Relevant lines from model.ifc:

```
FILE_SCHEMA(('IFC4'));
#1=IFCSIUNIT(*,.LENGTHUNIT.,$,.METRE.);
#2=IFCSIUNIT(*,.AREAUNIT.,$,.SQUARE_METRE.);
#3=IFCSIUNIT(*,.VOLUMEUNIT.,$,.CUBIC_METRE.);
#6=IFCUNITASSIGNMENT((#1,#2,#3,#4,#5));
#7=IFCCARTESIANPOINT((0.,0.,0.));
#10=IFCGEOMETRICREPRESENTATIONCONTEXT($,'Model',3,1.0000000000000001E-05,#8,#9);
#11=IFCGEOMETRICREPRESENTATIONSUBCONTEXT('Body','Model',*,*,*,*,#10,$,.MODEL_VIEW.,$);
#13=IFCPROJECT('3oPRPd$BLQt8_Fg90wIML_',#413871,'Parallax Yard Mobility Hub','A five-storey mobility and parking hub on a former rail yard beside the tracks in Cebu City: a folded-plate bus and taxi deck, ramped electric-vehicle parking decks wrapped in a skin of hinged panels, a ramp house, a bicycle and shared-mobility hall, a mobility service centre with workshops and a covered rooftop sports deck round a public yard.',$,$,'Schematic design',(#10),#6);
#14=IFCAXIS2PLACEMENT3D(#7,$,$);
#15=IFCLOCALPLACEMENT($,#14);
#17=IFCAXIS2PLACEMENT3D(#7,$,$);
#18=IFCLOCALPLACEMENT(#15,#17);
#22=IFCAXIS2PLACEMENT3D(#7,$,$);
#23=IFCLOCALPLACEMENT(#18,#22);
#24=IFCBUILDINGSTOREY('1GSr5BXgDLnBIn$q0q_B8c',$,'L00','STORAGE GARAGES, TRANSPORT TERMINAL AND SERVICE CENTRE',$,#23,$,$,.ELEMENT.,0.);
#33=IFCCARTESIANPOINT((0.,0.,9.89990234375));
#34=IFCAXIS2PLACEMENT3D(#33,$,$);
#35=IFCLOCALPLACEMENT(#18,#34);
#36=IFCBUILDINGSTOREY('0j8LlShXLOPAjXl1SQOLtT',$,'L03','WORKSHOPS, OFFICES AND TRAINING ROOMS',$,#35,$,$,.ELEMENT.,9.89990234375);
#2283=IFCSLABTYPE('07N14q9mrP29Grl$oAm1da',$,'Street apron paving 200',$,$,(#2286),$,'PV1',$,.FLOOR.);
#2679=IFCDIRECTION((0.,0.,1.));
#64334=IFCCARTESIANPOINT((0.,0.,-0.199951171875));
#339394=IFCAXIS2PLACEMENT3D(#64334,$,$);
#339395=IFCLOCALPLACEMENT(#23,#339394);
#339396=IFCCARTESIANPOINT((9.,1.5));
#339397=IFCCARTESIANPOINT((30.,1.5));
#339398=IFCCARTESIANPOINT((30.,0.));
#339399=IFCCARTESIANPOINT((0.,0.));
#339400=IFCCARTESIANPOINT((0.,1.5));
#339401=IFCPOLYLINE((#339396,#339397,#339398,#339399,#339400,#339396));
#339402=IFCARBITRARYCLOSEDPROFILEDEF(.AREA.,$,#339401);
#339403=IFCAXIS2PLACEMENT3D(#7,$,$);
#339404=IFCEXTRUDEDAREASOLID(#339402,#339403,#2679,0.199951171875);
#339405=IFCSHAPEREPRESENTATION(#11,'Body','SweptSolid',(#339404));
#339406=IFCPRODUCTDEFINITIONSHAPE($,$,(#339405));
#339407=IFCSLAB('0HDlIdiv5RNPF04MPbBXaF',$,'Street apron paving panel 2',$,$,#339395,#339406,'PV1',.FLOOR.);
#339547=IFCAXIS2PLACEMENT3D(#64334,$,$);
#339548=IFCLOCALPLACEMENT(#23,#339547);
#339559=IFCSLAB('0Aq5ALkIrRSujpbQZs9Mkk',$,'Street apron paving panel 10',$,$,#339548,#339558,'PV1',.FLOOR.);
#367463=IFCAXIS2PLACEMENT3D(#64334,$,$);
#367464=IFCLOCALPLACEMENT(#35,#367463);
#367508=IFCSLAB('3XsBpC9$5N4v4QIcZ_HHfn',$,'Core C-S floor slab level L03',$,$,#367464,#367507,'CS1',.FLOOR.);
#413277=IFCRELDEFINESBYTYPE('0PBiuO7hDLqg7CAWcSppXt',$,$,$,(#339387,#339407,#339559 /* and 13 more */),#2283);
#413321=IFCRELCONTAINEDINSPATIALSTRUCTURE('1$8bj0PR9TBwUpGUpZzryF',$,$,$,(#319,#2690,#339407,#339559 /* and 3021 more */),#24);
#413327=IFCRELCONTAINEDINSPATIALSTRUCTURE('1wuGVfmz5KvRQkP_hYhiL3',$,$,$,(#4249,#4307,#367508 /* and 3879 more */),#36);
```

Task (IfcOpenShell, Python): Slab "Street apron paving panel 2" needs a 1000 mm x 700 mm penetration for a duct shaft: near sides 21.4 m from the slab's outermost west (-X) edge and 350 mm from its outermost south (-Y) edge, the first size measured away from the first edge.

```python
import numpy as np
import ifcopenshell
import ifcopenshell.api.feature
import ifcopenshell.api.geometry
import ifcopenshell.api.root
import ifcopenshell.geom
import ifcopenshell.util.placement
import ifcopenshell.util.representation
import ifcopenshell.util.shape
import ifcopenshell.util.unit

model = ifcopenshell.open("model.ifc")
unit_scale = ifcopenshell.util.unit.calculate_unit_scale(model)
settings = ifcopenshell.geom.settings()


def volume(element):
    """Net volume in cubic metres, openings subtracted."""
    shape = ifcopenshell.geom.create_shape(settings, element)
    return ifcopenshell.util.shape.get_volume(shape.geometry)


slab = model.by_guid("0HDlIdiv5RNPF04MPbBXaF")
before = volume(slab)

# Extent in the slab's own axes, in metres. The edges named are its -X and -Y sides.
slab_shape = ifcopenshell.geom.create_shape(settings, slab)
vertices = ifcopenshell.util.shape.get_vertices(slab_shape.geometry)
x_min, y_min, bottom = vertices.min(axis=0)
top = vertices[:, 2].max()

opening = ifcopenshell.api.root.create_entity(model, ifc_class="IfcOpeningElement", name="Duct shaft opening", predefined_type="OPENING")
context = ifcopenshell.util.representation.get_context(model, "Model", "Body", "MODEL_VIEW")
width, depth = 1, 0.7
outline = [(0.0, 0.0), (width, 0.0), (width, depth), (0.0, depth), (0.0, 0.0)]
# Overshoot both faces by 50 mm so the cut is clean.
shape = ifcopenshell.api.geometry.add_slab_representation(
    model, context=context, depth=top - bottom + 0.1, polyline=outline
)
ifcopenshell.api.geometry.assign_representation(model, product=opening, representation=shape)

matrix = ifcopenshell.util.placement.get_local_placement(slab.ObjectPlacement)
matrix[:, 3] = matrix @ np.append(np.array([x_min + 21.4, y_min + 0.35, bottom - 0.05]) / unit_scale, 1.0)
ifcopenshell.api.geometry.edit_object_placement(model, product=opening, matrix=matrix, is_si=False)
ifcopenshell.api.feature.add_feature(model, feature=opening, element=slab)

after = volume(slab)

print(f"slab volume {before:.3f} -> {after:.3f} m3")

model.write("model_v2.ifc")
```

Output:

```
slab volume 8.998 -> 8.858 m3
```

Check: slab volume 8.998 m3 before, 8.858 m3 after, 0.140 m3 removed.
